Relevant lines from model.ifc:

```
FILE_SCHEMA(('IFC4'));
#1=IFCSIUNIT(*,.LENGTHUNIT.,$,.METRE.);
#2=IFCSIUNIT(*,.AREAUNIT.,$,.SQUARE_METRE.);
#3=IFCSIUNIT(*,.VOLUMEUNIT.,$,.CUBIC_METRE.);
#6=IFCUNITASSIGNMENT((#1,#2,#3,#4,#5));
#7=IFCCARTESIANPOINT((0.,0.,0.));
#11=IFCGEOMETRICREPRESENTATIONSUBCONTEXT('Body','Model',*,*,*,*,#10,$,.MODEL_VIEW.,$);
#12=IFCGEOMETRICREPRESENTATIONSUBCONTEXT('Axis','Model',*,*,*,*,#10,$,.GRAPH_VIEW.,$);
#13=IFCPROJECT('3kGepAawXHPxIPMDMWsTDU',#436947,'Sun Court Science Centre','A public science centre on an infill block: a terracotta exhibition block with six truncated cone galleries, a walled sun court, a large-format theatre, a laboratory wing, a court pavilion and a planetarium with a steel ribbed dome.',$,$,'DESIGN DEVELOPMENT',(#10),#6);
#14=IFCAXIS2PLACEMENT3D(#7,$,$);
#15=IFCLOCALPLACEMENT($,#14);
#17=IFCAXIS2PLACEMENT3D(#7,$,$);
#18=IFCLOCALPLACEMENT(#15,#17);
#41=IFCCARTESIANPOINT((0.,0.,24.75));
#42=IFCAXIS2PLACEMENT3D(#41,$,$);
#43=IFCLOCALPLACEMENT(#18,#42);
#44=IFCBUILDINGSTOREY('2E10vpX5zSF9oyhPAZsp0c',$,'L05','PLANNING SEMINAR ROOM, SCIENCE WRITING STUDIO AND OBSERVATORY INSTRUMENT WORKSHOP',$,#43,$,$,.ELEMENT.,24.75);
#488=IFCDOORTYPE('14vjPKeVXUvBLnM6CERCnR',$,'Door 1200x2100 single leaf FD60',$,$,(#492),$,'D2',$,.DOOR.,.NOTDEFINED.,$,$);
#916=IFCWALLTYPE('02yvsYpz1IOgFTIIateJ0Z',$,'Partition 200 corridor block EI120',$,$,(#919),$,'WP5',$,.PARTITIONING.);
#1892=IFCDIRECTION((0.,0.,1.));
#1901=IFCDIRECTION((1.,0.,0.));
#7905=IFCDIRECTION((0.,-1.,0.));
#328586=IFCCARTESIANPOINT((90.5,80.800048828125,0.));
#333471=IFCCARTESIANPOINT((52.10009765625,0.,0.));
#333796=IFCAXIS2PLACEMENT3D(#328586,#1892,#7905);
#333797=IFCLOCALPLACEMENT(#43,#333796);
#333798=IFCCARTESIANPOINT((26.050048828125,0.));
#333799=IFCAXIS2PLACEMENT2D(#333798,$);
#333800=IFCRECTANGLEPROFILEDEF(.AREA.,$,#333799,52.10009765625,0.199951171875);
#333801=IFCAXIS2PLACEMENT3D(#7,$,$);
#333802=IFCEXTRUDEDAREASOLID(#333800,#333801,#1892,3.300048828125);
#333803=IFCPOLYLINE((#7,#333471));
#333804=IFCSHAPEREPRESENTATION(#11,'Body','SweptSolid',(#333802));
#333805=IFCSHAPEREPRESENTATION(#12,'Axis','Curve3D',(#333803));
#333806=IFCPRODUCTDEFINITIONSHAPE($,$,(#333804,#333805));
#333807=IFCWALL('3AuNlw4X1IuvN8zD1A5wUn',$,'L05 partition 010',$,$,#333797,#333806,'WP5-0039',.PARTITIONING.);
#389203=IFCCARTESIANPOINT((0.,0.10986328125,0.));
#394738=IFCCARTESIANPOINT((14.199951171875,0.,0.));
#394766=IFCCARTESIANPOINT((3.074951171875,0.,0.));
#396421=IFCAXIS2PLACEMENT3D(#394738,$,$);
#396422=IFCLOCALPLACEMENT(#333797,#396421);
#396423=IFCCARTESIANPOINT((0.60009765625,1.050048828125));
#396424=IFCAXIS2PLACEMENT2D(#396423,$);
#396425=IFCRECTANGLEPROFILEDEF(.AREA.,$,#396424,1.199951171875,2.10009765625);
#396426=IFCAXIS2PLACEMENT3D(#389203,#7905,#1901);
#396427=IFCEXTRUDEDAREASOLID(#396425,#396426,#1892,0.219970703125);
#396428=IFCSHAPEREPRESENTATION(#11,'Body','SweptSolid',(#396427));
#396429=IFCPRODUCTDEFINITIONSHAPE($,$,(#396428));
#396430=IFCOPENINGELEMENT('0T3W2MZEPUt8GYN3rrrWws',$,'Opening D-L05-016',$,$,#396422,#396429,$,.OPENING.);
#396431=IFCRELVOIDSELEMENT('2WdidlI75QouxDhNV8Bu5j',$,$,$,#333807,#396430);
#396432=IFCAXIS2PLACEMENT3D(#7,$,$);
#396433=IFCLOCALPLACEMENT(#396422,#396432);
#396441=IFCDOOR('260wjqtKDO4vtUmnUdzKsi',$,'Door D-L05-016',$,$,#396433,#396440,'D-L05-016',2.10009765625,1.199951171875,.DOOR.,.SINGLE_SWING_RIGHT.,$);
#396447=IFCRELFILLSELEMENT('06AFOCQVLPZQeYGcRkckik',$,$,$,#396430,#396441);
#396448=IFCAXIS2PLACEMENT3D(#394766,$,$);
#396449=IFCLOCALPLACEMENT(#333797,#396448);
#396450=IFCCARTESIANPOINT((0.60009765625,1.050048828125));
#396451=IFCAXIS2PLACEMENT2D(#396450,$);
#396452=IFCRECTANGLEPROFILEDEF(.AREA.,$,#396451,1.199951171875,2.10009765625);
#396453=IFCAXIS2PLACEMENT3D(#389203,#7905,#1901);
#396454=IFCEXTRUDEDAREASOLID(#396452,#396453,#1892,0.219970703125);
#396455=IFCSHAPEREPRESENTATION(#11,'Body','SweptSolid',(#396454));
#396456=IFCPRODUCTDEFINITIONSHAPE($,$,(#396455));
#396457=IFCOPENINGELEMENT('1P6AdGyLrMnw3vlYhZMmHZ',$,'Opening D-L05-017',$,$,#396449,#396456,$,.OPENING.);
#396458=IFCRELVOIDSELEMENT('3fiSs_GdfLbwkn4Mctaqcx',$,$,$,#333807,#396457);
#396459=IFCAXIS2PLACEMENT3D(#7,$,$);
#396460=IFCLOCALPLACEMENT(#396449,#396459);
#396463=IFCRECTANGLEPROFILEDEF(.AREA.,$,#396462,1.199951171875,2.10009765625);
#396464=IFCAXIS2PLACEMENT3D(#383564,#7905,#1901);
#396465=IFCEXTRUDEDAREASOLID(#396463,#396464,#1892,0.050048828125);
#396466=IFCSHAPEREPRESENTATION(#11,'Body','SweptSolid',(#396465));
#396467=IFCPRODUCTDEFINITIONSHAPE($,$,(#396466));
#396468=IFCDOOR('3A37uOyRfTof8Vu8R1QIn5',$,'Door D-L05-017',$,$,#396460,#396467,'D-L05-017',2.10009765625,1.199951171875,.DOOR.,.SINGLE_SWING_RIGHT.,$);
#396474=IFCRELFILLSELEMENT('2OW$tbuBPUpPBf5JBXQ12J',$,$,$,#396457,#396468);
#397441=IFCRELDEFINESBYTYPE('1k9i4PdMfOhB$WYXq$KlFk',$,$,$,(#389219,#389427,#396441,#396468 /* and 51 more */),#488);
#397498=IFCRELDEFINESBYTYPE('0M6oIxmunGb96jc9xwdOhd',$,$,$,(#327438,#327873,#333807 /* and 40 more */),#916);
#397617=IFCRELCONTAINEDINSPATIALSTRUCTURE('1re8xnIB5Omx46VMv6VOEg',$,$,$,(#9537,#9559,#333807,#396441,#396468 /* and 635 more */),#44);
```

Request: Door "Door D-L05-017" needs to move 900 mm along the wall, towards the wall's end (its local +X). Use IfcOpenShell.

```python
import ifcopenshell
import ifcopenshell.api.geometry
import ifcopenshell.util.placement
import ifcopenshell.util.unit

model = ifcopenshell.open("model.ifc")
unit_scale = ifcopenshell.util.unit.calculate_unit_scale(model)

door = model.by_guid("3A37uOyRfTof8Vu8R1QIn5")
opening = door.FillsVoids[0].RelatingOpeningElement
wall = opening.VoidsElements[0].RelatingBuildingElement

wall_matrix = ifcopenshell.util.placement.get_local_placement(wall.ObjectPlacement)
shift = wall_matrix[:3, 0] * 0.9 / unit_scale
before = ifcopenshell.util.placement.get_local_placement(door.ObjectPlacement)[:3, 3].copy()

# The door is placed relative to its opening, so it follows when the opening moves.
matrix = ifcopenshell.util.placement.get_local_placement(opening.ObjectPlacement)
matrix[:3, 3] += shift
ifcopenshell.api.geometry.edit_object_placement(
    model, product=opening, matrix=matrix, is_si=False, should_transform_children=True
)

after = ifcopenshell.util.placement.get_local_placement(door.ObjectPlacement)[:3, 3]
print("door moved by", (after - before).round(3) + 0.0)

model.write("model_rev.ifc")
```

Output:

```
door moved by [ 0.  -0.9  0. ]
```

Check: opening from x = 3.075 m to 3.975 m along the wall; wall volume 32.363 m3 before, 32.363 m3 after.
